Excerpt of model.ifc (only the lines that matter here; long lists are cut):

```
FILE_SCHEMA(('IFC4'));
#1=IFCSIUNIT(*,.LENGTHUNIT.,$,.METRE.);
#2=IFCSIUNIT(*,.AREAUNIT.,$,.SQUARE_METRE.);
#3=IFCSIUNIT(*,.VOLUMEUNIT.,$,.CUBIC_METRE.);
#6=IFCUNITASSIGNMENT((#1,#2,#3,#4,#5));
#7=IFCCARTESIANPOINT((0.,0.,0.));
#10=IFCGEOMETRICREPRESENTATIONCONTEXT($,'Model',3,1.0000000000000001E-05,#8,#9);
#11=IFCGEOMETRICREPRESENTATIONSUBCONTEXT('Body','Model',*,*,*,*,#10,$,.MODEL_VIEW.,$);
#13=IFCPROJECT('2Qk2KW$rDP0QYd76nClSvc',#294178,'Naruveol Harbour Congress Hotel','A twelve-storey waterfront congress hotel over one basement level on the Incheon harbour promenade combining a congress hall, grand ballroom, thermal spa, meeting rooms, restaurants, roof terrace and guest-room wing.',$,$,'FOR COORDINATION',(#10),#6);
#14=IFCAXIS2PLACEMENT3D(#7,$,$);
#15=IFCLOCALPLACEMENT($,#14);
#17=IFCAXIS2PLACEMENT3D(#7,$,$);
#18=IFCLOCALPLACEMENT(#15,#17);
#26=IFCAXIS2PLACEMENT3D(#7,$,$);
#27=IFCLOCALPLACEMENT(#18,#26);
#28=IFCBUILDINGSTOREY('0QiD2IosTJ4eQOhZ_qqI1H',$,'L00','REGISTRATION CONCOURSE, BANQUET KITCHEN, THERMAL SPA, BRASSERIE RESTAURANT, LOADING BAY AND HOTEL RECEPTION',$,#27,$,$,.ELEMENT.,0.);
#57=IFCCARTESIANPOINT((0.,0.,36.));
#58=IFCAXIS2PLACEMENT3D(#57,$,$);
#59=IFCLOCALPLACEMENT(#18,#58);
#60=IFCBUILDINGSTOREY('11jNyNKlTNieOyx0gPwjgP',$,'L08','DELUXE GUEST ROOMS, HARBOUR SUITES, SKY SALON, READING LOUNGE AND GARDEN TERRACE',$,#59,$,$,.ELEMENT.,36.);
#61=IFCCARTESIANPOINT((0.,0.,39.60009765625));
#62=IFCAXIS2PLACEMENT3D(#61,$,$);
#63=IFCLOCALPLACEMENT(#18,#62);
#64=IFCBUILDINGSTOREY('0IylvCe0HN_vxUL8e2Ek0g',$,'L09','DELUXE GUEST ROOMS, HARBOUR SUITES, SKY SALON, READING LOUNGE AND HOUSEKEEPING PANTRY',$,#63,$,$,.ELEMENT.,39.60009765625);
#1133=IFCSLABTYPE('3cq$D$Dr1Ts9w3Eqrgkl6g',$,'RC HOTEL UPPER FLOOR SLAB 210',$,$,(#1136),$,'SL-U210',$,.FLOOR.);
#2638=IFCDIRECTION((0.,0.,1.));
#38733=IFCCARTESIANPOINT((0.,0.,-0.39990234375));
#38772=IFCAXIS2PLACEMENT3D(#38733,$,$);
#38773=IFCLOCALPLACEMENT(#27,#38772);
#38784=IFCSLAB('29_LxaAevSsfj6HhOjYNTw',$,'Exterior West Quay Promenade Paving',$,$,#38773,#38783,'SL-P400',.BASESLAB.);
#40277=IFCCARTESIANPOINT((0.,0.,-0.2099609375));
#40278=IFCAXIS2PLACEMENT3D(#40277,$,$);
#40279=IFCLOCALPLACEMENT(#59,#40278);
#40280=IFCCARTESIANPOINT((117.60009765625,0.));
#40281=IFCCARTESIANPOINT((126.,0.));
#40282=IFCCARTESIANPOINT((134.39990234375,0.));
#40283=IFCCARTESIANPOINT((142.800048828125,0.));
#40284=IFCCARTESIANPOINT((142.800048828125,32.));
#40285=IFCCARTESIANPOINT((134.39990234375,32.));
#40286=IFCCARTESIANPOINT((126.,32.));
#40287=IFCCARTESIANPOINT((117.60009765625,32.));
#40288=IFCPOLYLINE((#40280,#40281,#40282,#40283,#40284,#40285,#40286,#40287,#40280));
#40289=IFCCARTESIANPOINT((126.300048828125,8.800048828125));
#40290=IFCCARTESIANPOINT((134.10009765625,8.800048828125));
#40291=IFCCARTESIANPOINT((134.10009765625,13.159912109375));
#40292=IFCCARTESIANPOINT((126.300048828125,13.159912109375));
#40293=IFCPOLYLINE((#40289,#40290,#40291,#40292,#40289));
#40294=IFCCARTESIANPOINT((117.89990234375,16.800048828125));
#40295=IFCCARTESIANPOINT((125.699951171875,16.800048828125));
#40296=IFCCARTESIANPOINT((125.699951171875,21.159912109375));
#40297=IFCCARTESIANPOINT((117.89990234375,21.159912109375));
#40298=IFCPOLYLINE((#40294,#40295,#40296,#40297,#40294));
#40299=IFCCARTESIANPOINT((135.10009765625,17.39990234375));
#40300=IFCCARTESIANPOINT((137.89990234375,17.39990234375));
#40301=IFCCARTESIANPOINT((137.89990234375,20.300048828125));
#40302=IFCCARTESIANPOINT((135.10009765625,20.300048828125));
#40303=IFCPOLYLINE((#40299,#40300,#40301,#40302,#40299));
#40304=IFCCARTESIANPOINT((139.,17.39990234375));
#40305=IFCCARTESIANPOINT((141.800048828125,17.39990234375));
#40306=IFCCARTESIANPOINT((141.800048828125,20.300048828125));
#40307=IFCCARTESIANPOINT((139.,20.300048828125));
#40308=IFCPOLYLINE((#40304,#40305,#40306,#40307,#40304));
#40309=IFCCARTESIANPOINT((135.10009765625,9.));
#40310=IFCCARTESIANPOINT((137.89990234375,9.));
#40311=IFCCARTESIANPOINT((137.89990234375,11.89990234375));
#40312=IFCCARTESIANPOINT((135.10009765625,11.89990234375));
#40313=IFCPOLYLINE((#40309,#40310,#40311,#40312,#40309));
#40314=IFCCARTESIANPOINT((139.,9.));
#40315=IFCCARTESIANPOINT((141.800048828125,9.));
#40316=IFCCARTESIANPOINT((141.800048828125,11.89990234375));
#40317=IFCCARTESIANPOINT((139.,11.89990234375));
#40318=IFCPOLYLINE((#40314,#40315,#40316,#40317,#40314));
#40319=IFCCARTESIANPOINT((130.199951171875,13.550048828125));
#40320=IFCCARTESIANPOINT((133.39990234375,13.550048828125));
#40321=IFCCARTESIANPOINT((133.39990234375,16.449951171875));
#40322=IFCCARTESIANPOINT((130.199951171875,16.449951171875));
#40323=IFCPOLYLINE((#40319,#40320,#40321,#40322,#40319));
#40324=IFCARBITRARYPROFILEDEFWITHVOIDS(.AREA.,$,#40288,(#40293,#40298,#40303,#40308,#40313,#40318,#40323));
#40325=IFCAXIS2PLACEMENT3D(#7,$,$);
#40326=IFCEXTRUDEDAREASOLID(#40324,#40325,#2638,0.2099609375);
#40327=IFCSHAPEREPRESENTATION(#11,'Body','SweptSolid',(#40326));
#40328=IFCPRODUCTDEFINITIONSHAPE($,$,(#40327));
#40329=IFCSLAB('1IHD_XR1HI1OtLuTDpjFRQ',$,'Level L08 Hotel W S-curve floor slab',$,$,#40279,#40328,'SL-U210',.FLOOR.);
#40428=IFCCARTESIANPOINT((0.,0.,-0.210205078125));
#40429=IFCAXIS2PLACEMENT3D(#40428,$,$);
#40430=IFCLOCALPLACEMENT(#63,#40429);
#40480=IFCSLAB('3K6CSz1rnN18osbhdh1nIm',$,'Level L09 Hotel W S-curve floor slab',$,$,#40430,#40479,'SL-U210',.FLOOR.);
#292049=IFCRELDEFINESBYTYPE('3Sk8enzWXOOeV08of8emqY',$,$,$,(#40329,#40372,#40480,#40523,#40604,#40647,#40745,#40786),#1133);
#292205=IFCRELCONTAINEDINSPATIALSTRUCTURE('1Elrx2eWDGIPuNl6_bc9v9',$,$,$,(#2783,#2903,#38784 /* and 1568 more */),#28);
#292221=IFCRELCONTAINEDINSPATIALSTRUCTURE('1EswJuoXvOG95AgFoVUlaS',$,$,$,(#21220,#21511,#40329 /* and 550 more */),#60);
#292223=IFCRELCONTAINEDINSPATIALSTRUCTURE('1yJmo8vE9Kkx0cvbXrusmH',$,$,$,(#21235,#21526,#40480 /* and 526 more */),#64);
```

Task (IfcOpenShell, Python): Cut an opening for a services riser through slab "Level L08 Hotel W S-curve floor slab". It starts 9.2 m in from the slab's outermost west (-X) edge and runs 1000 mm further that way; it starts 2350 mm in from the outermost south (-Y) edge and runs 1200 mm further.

```python
import numpy as np
import ifcopenshell
import ifcopenshell.api.feature
import ifcopenshell.api.geometry
import ifcopenshell.api.root
import ifcopenshell.geom
import ifcopenshell.util.placement
import ifcopenshell.util.representation
import ifcopenshell.util.shape
import ifcopenshell.util.unit

model = ifcopenshell.open("model.ifc")
unit_scale = ifcopenshell.util.unit.calculate_unit_scale(model)
settings = ifcopenshell.geom.settings()


def volume(element):
    """Net volume in cubic metres, openings subtracted."""
    shape = ifcopenshell.geom.create_shape(settings, element)
    return ifcopenshell.util.shape.get_volume(shape.geometry)


slab = model.by_guid("1IHD_XR1HI1OtLuTDpjFRQ")
before = volume(slab)

# Extent in the slab's own axes, in metres. The edges named are its -X and -Y sides.
slab_shape = ifcopenshell.geom.create_shape(settings, slab)
vertices = ifcopenshell.util.shape.get_vertices(slab_shape.geometry)
x_min, y_min, bottom = vertices.min(axis=0)
top = vertices[:, 2].max()

opening = ifcopenshell.api.root.create_entity(model, ifc_class="IfcOpeningElement", name="Services riser opening", predefined_type="OPENING")
context = ifcopenshell.util.representation.get_context(model, "Model", "Body", "MODEL_VIEW")
width, depth = 1, 1.2
outline = [(0.0, 0.0), (width, 0.0), (width, depth), (0.0, depth), (0.0, 0.0)]
# Overshoot both faces by 50 mm so the cut is clean.
shape = ifcopenshell.api.geometry.add_slab_representation(
    model, context=context, depth=top - bottom + 0.1, polyline=outline
)
ifcopenshell.api.geometry.assign_representation(model, product=opening, representation=shape)

matrix = ifcopenshell.util.placement.get_local_placement(slab.ObjectPlacement)
matrix[:, 3] = matrix @ np.append(np.array([x_min + 9.2, y_min + 2.35, bottom - 0.05]) / unit_scale, 1.0)
ifcopenshell.api.geometry.edit_object_placement(model, product=opening, matrix=matrix, is_si=False)
ifcopenshell.api.feature.add_feature(model, feature=opening, element=slab)

after = volume(slab)

print(f"slab volume {before:.3f} -> {after:.3f} m3")

model.write("model_v2.ifc")
```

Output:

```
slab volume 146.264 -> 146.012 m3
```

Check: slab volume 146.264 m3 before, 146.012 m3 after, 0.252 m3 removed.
